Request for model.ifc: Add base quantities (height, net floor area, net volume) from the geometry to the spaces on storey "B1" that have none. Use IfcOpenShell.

First a look at what the model holds.

```python
import ifcopenshell
import ifcopenshell.util.element
import ifcopenshell.util.unit

model = ifcopenshell.open("model.ifc")
print(model.schema)
for unit_type in ("LENGTHUNIT", "AREAUNIT", "VOLUMEUNIT"):
    print(unit_type, ifcopenshell.util.unit.calculate_unit_scale(model, unit_type))
storey = next(s for s in model.by_type("IfcBuildingStorey") if s.Name == "B1")
spaces = [e for e in ifcopenshell.util.element.get_decomposition(storey) if e.is_a("IfcSpace")]
for e in sorted(spaces, key=lambda e: e.id()):
    print(e.id(), e.is_a(), e.Name, list(ifcopenshell.util.element.get_psets(e, qtos_only=True)), sep=" | ")
```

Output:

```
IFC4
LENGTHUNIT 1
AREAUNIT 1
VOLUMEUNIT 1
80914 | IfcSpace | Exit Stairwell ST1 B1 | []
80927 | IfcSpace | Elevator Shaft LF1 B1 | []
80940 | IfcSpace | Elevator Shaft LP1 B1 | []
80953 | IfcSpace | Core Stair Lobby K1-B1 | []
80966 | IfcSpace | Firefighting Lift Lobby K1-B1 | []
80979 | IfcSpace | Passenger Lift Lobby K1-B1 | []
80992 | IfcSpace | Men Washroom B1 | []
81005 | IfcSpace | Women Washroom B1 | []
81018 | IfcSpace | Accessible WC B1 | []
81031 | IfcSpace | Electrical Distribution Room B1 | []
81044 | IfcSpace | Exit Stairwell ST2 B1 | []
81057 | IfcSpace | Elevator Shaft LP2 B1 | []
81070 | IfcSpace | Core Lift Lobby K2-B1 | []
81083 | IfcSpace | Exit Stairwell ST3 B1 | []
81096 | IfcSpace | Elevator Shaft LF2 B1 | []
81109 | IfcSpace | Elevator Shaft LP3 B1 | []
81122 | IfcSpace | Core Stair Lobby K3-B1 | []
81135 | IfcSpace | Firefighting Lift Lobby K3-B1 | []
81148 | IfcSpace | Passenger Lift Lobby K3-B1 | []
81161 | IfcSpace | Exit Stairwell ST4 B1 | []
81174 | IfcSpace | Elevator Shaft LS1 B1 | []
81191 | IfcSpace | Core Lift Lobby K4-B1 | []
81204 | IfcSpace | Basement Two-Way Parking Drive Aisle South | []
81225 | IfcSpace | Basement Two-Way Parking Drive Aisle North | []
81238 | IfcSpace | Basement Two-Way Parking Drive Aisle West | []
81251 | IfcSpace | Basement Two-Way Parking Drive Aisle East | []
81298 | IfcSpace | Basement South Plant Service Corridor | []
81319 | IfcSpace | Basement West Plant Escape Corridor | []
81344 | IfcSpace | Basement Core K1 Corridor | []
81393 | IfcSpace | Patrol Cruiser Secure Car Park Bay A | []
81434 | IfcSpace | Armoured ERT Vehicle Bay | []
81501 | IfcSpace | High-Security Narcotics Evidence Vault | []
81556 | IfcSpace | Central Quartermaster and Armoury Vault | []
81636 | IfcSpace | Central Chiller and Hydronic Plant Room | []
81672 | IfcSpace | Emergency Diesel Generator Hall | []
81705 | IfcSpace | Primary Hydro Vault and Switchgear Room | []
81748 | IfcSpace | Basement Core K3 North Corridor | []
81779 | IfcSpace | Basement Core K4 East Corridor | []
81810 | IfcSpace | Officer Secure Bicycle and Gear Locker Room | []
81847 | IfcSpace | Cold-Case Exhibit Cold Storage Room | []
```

```python
import ifcopenshell
import ifcopenshell.api.pset
import ifcopenshell.geom
import ifcopenshell.util.element
import ifcopenshell.util.shape
import ifcopenshell.util.unit

model = ifcopenshell.open("model.ifc")
unit_scale = ifcopenshell.util.unit.calculate_unit_scale(model)
area_scale = ifcopenshell.util.unit.calculate_unit_scale(model, "AREAUNIT")
volume_scale = ifcopenshell.util.unit.calculate_unit_scale(model, "VOLUMEUNIT")
settings = ifcopenshell.geom.settings()

storey = next(s for s in model.by_type("IfcBuildingStorey") if s.Name == "B1")
spaces = [e for e in ifcopenshell.util.element.get_decomposition(storey) if e.is_a("IfcSpace")]

for e in sorted(spaces, key=lambda e: e.id()):
    if ifcopenshell.util.element.get_psets(e, qtos_only=True, should_inherit=False):
        continue
    # Geometry comes back in metres, in the element's own axes.
    shape = ifcopenshell.geom.create_shape(settings, e)
    values = {
        "Height": ifcopenshell.util.shape.get_z(shape.geometry) / unit_scale,
        "NetFloorArea": ifcopenshell.util.shape.get_footprint_area(shape.geometry) / area_scale,
        "NetVolume": ifcopenshell.util.shape.get_volume(shape.geometry) / volume_scale,
    }
    qto = ifcopenshell.api.pset.add_qto(model, product=e, name="Qto_SpaceBaseQuantities")
    ifcopenshell.api.pset.edit_qto(model, qto=qto, properties=values)
    print(e.id(), {k: round(v, 3) for k, v in values.items()})

model.write("model-out.ifc")
```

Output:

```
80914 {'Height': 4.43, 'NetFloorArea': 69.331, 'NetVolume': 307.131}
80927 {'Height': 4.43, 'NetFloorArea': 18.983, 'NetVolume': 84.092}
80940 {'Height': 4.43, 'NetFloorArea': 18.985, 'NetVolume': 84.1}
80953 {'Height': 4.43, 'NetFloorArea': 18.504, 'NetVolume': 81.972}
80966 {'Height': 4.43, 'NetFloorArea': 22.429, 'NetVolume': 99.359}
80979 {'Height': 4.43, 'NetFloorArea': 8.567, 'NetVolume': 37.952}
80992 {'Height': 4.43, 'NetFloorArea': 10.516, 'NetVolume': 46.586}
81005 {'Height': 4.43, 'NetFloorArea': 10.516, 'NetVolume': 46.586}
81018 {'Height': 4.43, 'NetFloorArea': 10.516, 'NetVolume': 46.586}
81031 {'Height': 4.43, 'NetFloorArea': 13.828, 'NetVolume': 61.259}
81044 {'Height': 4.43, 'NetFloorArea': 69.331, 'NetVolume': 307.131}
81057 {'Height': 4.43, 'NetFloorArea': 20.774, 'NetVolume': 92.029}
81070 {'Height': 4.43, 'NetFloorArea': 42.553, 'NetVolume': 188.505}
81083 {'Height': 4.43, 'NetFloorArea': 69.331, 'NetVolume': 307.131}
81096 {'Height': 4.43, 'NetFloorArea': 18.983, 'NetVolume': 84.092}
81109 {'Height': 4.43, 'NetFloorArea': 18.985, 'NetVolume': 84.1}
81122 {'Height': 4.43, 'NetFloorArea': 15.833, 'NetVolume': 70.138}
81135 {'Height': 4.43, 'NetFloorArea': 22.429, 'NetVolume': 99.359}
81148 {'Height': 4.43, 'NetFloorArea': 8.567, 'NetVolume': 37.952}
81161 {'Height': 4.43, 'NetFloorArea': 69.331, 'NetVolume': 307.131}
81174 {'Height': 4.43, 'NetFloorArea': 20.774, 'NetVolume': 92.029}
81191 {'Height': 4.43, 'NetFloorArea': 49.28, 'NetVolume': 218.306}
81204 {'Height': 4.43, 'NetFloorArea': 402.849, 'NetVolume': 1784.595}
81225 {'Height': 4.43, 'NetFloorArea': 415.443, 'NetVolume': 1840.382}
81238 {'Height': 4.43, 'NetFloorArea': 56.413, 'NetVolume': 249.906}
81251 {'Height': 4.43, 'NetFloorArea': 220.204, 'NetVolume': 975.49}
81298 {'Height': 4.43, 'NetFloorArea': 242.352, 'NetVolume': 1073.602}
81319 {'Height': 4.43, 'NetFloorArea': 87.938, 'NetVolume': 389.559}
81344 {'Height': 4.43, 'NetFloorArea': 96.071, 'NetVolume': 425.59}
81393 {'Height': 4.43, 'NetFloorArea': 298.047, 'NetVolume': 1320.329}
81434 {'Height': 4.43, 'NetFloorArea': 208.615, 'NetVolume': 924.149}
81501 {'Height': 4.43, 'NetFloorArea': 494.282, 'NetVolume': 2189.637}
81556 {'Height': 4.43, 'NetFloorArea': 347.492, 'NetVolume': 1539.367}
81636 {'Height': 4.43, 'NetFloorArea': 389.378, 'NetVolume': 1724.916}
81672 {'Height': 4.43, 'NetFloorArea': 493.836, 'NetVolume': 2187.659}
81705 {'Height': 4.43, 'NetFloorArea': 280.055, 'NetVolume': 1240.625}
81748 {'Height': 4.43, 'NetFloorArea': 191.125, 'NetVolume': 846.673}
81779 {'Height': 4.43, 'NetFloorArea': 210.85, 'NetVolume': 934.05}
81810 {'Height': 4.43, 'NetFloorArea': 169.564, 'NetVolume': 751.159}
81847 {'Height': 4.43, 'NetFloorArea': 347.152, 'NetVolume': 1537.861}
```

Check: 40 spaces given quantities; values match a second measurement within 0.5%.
